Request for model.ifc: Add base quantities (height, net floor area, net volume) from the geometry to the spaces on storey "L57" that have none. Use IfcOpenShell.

First a look at what the model holds.

```python
import ifcopenshell
import ifcopenshell.util.element
import ifcopenshell.util.unit

model = ifcopenshell.open("model.ifc")
print(model.schema)
for unit_type in ("LENGTHUNIT", "AREAUNIT", "VOLUMEUNIT"):
    print(unit_type, ifcopenshell.util.unit.calculate_unit_scale(model, unit_type))
storey = next(s for s in model.by_type("IfcBuildingStorey") if s.Name == "L57")
spaces = [e for e in ifcopenshell.util.element.get_decomposition(storey) if e.is_a("IfcSpace")]
for e in sorted(spaces, key=lambda e: e.id()):
    print(e.id(), e.is_a(), e.Name, list(ifcopenshell.util.element.get_psets(e, qtos_only=True)), sep=" | ")
```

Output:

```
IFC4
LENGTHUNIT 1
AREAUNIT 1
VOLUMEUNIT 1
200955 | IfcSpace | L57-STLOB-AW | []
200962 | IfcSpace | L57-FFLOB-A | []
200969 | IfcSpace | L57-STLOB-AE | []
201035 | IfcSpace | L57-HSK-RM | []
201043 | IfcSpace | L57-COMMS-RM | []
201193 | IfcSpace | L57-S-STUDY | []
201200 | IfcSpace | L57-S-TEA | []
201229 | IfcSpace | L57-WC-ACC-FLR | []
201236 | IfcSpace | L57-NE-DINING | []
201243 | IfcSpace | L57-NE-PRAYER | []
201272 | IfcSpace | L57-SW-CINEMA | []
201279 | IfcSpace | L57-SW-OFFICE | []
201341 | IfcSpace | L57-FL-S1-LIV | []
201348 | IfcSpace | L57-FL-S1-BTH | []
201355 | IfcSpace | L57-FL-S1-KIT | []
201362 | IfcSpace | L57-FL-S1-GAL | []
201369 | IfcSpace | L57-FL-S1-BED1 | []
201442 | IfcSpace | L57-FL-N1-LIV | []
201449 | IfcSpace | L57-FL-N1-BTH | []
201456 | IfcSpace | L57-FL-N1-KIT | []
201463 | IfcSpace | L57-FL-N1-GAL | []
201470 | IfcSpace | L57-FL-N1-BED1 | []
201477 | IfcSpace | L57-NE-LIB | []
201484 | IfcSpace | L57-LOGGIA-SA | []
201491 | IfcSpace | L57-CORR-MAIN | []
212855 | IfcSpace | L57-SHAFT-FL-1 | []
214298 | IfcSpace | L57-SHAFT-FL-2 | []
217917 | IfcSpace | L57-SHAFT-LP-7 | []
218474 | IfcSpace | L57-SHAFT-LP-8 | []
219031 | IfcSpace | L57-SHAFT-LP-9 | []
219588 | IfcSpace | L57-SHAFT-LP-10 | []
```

```python
import ifcopenshell
import ifcopenshell.api.pset
import ifcopenshell.geom
import ifcopenshell.util.element
import ifcopenshell.util.shape
import ifcopenshell.util.unit

model = ifcopenshell.open("model.ifc")
unit_scale = ifcopenshell.util.unit.calculate_unit_scale(model)
area_scale = ifcopenshell.util.unit.calculate_unit_scale(model, "AREAUNIT")
volume_scale = ifcopenshell.util.unit.calculate_unit_scale(model, "VOLUMEUNIT")
settings = ifcopenshell.geom.settings()

storey = next(s for s in model.by_type("IfcBuildingStorey") if s.Name == "L57")
spaces = [e for e in ifcopenshell.util.element.get_decomposition(storey) if e.is_a("IfcSpace")]

for e in sorted(spaces, key=lambda e: e.id()):
    if ifcopenshell.util.element.get_psets(e, qtos_only=True, should_inherit=False):
        continue
    # Geometry comes back in metres, in the element's own axes.
    shape = ifcopenshell.geom.create_shape(settings, e)
    values = {
        "Height": ifcopenshell.util.shape.get_z(shape.geometry) / unit_scale,
        "NetFloorArea": ifcopenshell.util.shape.get_footprint_area(shape.geometry) / area_scale,
        "NetVolume": ifcopenshell.util.shape.get_volume(shape.geometry) / volume_scale,
    }
    qto = ifcopenshell.api.pset.add_qto(model, product=e, name="Qto_SpaceBaseQuantities")
    ifcopenshell.api.pset.edit_qto(model, qto=qto, properties=values)
    print(e.id(), {k: round(v, 3) for k, v in values.items()})

model.write("model_v2.ifc")
```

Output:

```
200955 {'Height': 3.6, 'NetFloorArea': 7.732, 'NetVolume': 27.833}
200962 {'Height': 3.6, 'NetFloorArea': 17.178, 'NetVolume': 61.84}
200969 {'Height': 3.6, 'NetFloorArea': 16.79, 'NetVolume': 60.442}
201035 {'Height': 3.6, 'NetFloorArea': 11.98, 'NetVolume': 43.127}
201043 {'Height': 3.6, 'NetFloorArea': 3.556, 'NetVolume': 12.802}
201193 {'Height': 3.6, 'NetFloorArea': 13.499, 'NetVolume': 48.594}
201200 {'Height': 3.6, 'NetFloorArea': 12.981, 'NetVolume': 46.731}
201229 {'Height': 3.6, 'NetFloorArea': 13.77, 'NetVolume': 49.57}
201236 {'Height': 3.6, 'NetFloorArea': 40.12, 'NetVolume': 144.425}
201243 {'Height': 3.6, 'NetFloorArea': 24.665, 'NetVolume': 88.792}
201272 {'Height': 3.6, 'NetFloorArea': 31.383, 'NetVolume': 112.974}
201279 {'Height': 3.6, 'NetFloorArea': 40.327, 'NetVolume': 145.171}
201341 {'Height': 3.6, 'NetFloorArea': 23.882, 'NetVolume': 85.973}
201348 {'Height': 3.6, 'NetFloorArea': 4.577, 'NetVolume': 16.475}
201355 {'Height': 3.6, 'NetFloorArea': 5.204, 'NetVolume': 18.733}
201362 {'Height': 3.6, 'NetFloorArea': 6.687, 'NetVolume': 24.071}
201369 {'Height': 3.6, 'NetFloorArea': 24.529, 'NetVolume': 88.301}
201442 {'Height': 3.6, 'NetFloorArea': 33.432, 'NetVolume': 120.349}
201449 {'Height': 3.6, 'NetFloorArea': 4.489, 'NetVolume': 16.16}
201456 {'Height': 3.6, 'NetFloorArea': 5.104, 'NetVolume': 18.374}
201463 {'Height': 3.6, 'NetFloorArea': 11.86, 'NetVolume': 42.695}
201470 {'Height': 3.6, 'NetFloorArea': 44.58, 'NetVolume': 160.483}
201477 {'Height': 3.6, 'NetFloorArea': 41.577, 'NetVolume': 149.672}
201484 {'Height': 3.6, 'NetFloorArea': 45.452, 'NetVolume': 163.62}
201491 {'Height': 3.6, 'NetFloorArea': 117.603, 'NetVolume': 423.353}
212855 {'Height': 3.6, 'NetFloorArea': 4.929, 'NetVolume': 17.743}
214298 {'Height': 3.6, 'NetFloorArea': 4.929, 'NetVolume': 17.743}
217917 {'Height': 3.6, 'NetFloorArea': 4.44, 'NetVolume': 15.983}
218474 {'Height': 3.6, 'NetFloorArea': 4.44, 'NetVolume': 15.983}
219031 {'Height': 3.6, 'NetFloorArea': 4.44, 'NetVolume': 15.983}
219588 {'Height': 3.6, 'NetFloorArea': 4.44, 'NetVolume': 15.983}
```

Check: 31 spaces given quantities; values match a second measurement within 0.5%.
